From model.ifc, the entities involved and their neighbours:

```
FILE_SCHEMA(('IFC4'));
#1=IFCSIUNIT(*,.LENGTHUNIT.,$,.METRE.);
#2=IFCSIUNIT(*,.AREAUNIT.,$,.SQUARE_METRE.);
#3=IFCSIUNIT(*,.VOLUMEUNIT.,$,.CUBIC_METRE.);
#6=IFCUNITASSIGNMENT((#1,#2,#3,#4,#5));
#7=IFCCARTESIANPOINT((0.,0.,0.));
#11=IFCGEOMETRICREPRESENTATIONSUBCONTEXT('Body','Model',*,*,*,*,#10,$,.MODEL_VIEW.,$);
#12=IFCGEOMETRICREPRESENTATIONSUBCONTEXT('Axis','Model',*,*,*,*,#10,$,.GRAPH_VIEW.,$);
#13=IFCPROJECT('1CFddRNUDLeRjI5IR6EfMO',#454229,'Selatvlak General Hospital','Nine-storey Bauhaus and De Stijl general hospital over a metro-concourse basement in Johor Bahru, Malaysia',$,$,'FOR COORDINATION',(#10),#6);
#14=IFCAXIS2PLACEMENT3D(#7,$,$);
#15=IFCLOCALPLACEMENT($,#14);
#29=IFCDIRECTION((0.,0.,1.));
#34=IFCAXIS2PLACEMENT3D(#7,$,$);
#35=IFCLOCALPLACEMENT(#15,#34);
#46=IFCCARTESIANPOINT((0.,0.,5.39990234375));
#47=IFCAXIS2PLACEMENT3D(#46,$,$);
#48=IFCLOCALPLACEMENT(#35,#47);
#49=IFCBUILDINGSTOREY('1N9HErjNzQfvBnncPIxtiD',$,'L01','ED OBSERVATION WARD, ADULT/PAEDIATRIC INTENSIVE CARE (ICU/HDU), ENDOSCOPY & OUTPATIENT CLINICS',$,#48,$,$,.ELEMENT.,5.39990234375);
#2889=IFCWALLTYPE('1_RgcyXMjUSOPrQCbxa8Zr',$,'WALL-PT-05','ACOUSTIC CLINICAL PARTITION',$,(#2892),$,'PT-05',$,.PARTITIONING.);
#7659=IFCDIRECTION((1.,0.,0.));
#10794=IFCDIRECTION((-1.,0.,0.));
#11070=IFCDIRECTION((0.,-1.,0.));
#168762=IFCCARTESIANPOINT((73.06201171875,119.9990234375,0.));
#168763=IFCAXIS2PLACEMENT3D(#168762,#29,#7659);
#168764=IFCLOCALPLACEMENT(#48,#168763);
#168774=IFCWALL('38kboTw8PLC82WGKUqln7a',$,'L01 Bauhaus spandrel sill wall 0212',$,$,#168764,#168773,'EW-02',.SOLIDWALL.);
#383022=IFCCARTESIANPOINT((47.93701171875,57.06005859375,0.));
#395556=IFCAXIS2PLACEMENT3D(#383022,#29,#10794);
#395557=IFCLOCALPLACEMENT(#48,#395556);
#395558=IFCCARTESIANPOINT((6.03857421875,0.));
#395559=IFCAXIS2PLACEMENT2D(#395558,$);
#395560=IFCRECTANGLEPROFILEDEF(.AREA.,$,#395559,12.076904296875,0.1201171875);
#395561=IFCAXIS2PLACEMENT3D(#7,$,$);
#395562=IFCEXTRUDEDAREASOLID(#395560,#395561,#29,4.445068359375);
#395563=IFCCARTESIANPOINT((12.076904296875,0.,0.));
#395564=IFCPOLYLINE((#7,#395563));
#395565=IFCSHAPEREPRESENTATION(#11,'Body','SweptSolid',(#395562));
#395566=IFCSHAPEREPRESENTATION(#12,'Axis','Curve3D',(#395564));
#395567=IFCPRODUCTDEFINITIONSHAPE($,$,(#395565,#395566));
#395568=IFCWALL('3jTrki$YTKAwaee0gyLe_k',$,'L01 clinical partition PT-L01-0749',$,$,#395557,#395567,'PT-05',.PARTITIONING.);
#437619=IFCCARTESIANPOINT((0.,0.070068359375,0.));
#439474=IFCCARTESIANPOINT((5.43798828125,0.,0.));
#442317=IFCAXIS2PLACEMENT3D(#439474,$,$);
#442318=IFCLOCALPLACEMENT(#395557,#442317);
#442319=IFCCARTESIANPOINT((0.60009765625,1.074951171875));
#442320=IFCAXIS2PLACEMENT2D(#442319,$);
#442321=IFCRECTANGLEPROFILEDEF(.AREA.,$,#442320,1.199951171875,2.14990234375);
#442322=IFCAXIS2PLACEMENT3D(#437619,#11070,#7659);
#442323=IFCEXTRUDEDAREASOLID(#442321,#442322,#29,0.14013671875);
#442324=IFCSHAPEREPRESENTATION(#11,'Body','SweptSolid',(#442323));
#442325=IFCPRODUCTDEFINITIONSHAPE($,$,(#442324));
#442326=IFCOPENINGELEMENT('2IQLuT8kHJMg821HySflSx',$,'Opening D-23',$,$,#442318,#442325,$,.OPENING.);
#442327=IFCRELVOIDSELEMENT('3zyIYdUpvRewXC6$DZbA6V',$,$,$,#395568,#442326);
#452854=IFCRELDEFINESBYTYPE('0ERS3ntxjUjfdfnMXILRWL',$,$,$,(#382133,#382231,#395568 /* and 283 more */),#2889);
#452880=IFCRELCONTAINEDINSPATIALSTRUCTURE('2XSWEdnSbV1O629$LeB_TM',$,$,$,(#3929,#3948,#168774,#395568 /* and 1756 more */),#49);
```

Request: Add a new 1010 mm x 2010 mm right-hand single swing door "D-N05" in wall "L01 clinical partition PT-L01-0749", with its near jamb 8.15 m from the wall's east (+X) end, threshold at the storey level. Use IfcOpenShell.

```python
import numpy as np
import ifcopenshell
import ifcopenshell.api.feature
import ifcopenshell.api.geometry
import ifcopenshell.api.root
import ifcopenshell.api.spatial
import ifcopenshell.geom
import ifcopenshell.util.element
import ifcopenshell.util.placement
import ifcopenshell.util.representation
import ifcopenshell.util.shape
import ifcopenshell.util.unit

model = ifcopenshell.open("model.ifc")
unit_scale = ifcopenshell.util.unit.calculate_unit_scale(model)
settings = ifcopenshell.geom.settings()


def volume(element):
    """Net volume in cubic metres, openings subtracted."""
    shape = ifcopenshell.geom.create_shape(settings, element)
    return ifcopenshell.util.shape.get_volume(shape.geometry)


wall = model.by_guid("3jTrki$YTKAwaee0gyLe_k")
storey = ifcopenshell.util.element.get_container(wall, ifc_class="IfcBuildingStorey")
context = ifcopenshell.util.representation.get_context(model, "Model", "Body", "MODEL_VIEW")
before = volume(wall)

width, height, from_end, sill = 1.01, 2.01, 8.15, 0.0  # metres

# The wall runs along its own X axis, and the end named is its -X end.
wall_shape = ifcopenshell.geom.create_shape(settings, wall)
x, y, z = ifcopenshell.util.shape.get_vertices(wall_shape.geometry).T
start = x.min() + from_end
face, thickness = float(y.min()), float(y.max() - y.min())
wall_matrix = ifcopenshell.util.placement.get_local_placement(wall.ObjectPlacement)
level = ifcopenshell.util.placement.get_local_placement(storey.ObjectPlacement)[2, 3]


def in_wall(x, y):
    """Placement at x, y metres in the wall's axes, at sill height."""
    matrix = wall_matrix.copy()
    matrix[:, 3] = wall_matrix @ np.array([x / unit_scale, y / unit_scale, 0.0, 1.0])
    matrix[2, 3] = level + sill / unit_scale
    return matrix


# Opening: a box that overshoots both wall faces by 50 mm.
opening = ifcopenshell.api.root.create_entity(model, ifc_class="IfcOpeningElement", predefined_type="OPENING")
box = ifcopenshell.api.geometry.add_wall_representation(
    model, context=context, length=width, height=height, thickness=thickness + 0.1
)
ifcopenshell.api.geometry.assign_representation(model, product=opening, representation=box)
ifcopenshell.api.geometry.edit_object_placement(model, product=opening, matrix=in_wall(start, face - 0.05), is_si=False)
ifcopenshell.api.feature.add_feature(model, feature=opening, element=wall)

door = ifcopenshell.api.root.create_entity(model, ifc_class="IfcDoor", name="D-N05", predefined_type="DOOR")
door.OverallWidth, door.OverallHeight = width / unit_scale, height / unit_scale
door.OperationType = "SINGLE_SWING_RIGHT"
body = ifcopenshell.api.geometry.add_door_representation(
    model,
    context=context,
    overall_width=door.OverallWidth,
    overall_height=door.OverallHeight,
    operation_type="SINGLE_SWING_RIGHT",
    lining_properties={"LiningDepth": thickness / unit_scale, "ThresholdDepth": thickness / unit_scale},
)
ifcopenshell.api.geometry.assign_representation(model, product=door, representation=body)
ifcopenshell.api.spatial.assign_container(model, products=[door], relating_structure=storey)
ifcopenshell.api.feature.add_filling(model, opening=opening, element=door)

# The lining spans the wall, so the door starts at the wall face.
ifcopenshell.api.geometry.edit_object_placement(model, product=door, matrix=in_wall(start, face), is_si=False)

after = volume(wall)

print(f"wall volume {before:.3f} -> {after:.3f} m3")

model.write("model_edited.ifc")
```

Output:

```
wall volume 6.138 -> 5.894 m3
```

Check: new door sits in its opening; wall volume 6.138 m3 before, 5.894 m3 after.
